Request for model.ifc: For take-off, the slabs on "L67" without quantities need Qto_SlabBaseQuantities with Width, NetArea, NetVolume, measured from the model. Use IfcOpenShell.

First a look at what the model holds.

```python
import ifcopenshell
import ifcopenshell.util.element
import ifcopenshell.util.unit

model = ifcopenshell.open("model.ifc")
print(model.schema)
for unit_type in ("LENGTHUNIT", "AREAUNIT", "VOLUMEUNIT"):
    print(unit_type, ifcopenshell.util.unit.calculate_unit_scale(model, unit_type))
storey = next(s for s in model.by_type("IfcBuildingStorey") if s.Name == "L67")
slabs = [e for e in ifcopenshell.util.element.get_decomposition(storey) if e.is_a("IfcSlab")]
for e in sorted(slabs, key=lambda e: e.id()):
    print(e.id(), e.is_a(), e.Name, list(ifcopenshell.util.element.get_psets(e, qtos_only=True)), sep=" | ")
```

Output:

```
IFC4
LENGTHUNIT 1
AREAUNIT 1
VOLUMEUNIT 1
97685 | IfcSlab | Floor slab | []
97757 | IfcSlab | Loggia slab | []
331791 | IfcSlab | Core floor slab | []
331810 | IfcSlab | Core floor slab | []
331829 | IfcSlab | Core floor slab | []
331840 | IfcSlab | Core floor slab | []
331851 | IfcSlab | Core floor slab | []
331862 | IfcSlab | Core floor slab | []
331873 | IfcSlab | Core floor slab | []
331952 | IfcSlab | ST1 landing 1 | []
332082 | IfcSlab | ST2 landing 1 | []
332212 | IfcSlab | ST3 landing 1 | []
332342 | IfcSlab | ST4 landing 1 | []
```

```python
import ifcopenshell
import ifcopenshell.api.pset
import ifcopenshell.geom
import ifcopenshell.util.element
import ifcopenshell.util.shape
import ifcopenshell.util.unit

model = ifcopenshell.open("model.ifc")
unit_scale = ifcopenshell.util.unit.calculate_unit_scale(model)
area_scale = ifcopenshell.util.unit.calculate_unit_scale(model, "AREAUNIT")
volume_scale = ifcopenshell.util.unit.calculate_unit_scale(model, "VOLUMEUNIT")
settings = ifcopenshell.geom.settings()

storey = next(s for s in model.by_type("IfcBuildingStorey") if s.Name == "L67")
slabs = [e for e in ifcopenshell.util.element.get_decomposition(storey) if e.is_a("IfcSlab")]

for e in sorted(slabs, key=lambda e: e.id()):
    if ifcopenshell.util.element.get_psets(e, qtos_only=True, should_inherit=False):
        continue
    # Geometry comes back in metres, in the element's own axes.
    shape = ifcopenshell.geom.create_shape(settings, e)
    values = {
        "Width": ifcopenshell.util.shape.get_z(shape.geometry) / unit_scale,
        "NetArea": ifcopenshell.util.shape.get_footprint_area(shape.geometry) / area_scale,
        "NetVolume": ifcopenshell.util.shape.get_volume(shape.geometry) / volume_scale,
    }
    qto = ifcopenshell.api.pset.add_qto(model, product=e, name="Qto_SlabBaseQuantities")
    ifcopenshell.api.pset.edit_qto(model, qto=qto, properties=values)
    print(e.id(), {k: round(v, 3) for k, v in values.items()})

model.write("model_rev.ifc")
```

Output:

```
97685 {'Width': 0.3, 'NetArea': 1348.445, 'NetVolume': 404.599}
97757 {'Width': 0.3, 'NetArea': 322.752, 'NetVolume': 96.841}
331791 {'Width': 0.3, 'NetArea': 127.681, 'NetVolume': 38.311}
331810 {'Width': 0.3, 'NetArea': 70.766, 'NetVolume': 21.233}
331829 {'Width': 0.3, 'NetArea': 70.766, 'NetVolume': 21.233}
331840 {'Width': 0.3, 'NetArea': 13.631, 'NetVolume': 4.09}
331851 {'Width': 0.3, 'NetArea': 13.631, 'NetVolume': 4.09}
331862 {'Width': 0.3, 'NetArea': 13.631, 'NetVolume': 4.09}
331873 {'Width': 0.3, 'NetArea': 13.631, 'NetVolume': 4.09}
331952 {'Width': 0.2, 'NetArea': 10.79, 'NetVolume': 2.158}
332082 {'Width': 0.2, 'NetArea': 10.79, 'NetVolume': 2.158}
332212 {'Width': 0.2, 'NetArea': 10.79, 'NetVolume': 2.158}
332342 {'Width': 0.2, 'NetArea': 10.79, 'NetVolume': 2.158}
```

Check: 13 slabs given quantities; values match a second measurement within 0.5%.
